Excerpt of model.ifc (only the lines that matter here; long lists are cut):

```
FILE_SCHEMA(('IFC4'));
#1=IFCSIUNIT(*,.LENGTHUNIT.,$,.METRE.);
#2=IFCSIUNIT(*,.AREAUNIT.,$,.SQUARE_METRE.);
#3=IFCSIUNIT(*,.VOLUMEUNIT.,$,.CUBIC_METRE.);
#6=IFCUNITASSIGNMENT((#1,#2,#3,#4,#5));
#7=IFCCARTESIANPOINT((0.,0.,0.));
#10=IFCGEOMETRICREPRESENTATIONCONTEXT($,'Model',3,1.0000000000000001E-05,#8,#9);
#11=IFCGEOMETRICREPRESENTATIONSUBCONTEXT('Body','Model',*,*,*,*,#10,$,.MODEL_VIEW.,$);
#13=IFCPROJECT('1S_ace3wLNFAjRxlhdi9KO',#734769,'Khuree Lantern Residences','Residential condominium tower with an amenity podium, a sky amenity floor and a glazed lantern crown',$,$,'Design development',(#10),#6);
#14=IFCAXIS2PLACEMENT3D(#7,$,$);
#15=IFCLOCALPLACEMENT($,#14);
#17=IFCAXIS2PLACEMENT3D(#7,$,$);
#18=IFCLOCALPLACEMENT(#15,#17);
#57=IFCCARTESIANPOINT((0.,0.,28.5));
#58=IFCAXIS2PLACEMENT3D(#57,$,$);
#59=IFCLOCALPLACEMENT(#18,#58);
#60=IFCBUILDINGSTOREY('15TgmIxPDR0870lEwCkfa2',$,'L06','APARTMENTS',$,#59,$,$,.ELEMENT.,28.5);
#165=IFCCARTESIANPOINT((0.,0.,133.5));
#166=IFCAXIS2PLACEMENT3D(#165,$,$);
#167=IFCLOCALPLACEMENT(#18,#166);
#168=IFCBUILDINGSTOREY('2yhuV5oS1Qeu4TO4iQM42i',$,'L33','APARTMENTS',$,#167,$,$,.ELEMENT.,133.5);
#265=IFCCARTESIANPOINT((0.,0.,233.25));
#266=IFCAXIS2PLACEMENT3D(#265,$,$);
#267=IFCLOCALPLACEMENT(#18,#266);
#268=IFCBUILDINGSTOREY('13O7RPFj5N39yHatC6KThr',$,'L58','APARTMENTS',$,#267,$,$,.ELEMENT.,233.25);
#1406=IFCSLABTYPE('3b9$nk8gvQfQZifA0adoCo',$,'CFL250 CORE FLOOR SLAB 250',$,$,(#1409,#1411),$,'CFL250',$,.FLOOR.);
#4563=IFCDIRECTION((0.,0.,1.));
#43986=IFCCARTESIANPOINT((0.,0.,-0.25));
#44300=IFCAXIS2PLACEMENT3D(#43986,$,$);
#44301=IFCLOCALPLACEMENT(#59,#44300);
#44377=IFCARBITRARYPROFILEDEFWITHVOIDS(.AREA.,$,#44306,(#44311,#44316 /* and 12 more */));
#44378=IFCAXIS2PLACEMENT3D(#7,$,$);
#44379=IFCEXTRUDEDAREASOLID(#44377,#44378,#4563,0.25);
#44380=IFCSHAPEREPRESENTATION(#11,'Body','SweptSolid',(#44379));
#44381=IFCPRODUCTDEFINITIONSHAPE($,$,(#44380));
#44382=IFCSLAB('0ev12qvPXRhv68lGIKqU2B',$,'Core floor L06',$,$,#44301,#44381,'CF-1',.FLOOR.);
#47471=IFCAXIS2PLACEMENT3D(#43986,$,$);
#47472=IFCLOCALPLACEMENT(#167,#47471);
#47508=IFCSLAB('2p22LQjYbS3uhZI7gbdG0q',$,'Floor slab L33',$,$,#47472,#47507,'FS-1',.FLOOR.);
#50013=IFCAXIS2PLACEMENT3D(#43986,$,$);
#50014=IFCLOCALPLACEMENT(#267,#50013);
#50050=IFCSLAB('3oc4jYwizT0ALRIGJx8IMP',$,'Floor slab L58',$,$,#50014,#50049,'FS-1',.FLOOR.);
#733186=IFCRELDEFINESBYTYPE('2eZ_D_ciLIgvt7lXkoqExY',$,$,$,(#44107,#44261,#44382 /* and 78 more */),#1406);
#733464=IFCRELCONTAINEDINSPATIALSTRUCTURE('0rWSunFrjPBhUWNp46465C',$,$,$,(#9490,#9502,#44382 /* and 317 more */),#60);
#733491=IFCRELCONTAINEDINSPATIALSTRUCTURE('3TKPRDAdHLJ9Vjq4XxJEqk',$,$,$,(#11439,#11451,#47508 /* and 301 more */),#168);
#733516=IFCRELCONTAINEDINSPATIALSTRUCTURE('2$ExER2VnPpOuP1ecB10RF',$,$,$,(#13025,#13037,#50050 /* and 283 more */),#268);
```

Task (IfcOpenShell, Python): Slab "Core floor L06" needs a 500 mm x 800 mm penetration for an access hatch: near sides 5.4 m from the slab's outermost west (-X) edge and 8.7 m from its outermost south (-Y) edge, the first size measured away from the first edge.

```python
import numpy as np
import ifcopenshell
import ifcopenshell.api.feature
import ifcopenshell.api.geometry
import ifcopenshell.api.root
import ifcopenshell.geom
import ifcopenshell.util.placement
import ifcopenshell.util.representation
import ifcopenshell.util.shape
import ifcopenshell.util.unit

model = ifcopenshell.open("model.ifc")
unit_scale = ifcopenshell.util.unit.calculate_unit_scale(model)
settings = ifcopenshell.geom.settings()


def volume(element):
    """Net volume in cubic metres, openings subtracted."""
    shape = ifcopenshell.geom.create_shape(settings, element)
    return ifcopenshell.util.shape.get_volume(shape.geometry)


slab = model.by_guid("0ev12qvPXRhv68lGIKqU2B")
before = volume(slab)

# Extent in the slab's own axes, in metres. The edges named are its -X and -Y sides.
slab_shape = ifcopenshell.geom.create_shape(settings, slab)
vertices = ifcopenshell.util.shape.get_vertices(slab_shape.geometry)
x_min, y_min, bottom = vertices.min(axis=0)
top = vertices[:, 2].max()

opening = ifcopenshell.api.root.create_entity(model, ifc_class="IfcOpeningElement", name="Access hatch opening", predefined_type="OPENING")
context = ifcopenshell.util.representation.get_context(model, "Model", "Body", "MODEL_VIEW")
width, depth = 0.5, 0.8
outline = [(0.0, 0.0), (width, 0.0), (width, depth), (0.0, depth), (0.0, 0.0)]
# Overshoot both faces by 50 mm so the cut is clean.
shape = ifcopenshell.api.geometry.add_slab_representation(
    model, context=context, depth=top - bottom + 0.1, polyline=outline
)
ifcopenshell.api.geometry.assign_representation(model, product=opening, representation=shape)

matrix = ifcopenshell.util.placement.get_local_placement(slab.ObjectPlacement)
matrix[:, 3] = matrix @ np.append(np.array([x_min + 5.4, y_min + 8.7, bottom - 0.05]) / unit_scale, 1.0)
ifcopenshell.api.geometry.edit_object_placement(model, product=opening, matrix=matrix, is_si=False)
ifcopenshell.api.feature.add_feature(model, feature=opening, element=slab)

after = volume(slab)

print(f"slab volume {before:.3f} -> {after:.3f} m3")

model.write("model_v2.ifc")
```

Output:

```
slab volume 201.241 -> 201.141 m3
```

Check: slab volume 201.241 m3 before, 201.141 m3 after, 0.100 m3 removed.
